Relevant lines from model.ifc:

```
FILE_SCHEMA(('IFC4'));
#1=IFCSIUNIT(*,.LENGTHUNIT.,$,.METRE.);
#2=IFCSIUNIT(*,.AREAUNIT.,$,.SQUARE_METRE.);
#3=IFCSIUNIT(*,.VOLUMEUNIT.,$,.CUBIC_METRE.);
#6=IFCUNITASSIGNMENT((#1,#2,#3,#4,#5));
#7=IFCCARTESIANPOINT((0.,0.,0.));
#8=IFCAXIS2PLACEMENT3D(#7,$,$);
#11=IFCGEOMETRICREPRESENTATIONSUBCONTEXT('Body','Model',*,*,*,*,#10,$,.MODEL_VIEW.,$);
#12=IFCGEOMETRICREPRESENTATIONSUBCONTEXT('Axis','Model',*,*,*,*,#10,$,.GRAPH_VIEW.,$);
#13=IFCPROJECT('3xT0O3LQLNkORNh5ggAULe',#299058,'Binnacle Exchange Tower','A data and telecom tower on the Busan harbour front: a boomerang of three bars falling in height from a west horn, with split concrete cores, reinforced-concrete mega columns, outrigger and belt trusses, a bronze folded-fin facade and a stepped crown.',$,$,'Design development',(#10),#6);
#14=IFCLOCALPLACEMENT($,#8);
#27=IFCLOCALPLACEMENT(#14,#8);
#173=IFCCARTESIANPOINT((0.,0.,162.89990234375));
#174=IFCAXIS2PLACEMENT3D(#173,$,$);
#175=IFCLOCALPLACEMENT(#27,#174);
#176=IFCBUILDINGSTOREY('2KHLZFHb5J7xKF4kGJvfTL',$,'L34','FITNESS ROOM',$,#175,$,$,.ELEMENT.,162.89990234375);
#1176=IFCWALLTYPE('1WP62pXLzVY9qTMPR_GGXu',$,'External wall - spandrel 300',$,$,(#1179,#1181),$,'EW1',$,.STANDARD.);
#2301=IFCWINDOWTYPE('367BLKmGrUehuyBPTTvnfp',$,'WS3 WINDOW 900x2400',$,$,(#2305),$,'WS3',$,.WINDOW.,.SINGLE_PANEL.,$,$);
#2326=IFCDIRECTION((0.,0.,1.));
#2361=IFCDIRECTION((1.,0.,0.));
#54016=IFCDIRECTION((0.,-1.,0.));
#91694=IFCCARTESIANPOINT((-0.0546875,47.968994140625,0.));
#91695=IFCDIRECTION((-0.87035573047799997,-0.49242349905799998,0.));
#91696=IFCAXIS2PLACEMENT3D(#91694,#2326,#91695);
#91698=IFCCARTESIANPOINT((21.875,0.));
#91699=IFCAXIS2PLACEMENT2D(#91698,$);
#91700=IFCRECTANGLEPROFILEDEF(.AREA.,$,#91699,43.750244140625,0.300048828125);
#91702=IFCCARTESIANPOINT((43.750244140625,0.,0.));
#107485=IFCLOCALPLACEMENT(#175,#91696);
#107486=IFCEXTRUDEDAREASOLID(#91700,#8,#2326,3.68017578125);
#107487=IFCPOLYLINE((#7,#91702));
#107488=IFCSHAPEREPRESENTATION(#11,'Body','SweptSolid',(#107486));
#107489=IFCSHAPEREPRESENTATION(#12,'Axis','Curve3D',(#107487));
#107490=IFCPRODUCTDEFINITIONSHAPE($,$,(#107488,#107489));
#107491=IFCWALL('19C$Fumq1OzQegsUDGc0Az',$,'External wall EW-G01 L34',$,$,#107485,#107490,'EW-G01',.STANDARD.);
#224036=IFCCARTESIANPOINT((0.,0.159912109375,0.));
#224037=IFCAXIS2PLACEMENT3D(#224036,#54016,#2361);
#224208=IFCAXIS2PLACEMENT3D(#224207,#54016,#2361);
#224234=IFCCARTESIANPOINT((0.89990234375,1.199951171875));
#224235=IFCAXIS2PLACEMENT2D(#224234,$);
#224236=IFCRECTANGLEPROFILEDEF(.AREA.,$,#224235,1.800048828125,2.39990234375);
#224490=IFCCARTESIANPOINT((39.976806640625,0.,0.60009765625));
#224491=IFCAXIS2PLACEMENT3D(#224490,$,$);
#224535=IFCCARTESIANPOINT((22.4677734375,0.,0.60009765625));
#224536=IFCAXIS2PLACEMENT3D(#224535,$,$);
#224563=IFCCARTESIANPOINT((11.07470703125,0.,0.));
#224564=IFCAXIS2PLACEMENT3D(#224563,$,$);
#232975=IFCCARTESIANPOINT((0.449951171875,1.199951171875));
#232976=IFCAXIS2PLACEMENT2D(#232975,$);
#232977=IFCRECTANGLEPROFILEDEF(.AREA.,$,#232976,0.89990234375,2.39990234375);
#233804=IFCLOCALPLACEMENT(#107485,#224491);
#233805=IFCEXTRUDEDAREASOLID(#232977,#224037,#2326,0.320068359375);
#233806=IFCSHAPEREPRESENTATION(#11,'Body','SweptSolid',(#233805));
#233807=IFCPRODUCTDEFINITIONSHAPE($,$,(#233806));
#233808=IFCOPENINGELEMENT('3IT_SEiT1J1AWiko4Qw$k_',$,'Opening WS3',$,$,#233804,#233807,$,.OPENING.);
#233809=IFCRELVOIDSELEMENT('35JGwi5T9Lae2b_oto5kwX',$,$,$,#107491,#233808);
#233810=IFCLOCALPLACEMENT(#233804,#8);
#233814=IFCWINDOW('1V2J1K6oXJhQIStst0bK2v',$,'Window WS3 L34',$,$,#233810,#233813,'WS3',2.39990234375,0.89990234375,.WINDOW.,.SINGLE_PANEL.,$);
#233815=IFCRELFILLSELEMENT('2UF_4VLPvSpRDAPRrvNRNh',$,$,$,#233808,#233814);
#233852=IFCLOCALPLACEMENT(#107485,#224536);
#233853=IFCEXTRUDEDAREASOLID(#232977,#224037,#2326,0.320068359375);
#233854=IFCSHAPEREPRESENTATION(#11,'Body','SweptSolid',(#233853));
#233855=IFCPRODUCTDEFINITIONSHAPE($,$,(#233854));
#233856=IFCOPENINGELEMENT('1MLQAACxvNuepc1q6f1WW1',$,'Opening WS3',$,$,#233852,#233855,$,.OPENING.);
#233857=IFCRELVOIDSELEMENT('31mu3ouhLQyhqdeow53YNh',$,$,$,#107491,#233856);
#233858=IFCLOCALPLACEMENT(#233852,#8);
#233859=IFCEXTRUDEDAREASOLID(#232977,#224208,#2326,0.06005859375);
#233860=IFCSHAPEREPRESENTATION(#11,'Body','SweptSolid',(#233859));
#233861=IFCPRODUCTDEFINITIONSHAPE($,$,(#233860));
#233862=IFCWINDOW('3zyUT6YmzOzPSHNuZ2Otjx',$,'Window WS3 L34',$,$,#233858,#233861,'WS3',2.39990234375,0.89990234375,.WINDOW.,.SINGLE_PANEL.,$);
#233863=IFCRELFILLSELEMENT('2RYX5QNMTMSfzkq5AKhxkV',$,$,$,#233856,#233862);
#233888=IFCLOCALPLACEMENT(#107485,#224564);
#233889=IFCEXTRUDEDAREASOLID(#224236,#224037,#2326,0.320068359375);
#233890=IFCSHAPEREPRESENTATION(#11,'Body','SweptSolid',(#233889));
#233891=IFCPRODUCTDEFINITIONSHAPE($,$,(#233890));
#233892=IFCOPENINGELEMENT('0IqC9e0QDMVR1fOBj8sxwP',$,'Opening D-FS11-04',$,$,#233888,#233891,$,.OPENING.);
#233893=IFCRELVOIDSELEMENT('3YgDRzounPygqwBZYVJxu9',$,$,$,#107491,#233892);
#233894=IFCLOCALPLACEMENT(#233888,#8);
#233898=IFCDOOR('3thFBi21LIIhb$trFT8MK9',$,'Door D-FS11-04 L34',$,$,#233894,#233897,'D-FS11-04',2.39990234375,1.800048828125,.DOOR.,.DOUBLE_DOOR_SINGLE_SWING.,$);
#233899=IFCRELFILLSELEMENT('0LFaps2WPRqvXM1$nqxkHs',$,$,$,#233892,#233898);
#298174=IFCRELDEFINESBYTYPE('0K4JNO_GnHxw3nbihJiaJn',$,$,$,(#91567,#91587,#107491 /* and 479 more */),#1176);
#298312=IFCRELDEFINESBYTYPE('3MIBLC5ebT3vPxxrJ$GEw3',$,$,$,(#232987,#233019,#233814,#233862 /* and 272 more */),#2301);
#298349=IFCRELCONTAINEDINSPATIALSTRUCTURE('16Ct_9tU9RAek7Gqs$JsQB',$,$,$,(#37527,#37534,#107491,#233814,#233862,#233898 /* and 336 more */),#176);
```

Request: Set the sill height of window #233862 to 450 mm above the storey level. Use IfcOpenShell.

```python
import numpy as np
import ifcopenshell
import ifcopenshell.api.geometry
import ifcopenshell.geom
import ifcopenshell.util.element
import ifcopenshell.util.placement
import ifcopenshell.util.shape
import ifcopenshell.util.unit

model = ifcopenshell.open("model.ifc")
unit_scale = ifcopenshell.util.unit.calculate_unit_scale(model)

window = model.by_id(233862)
opening = window.FillsVoids[0].RelatingOpeningElement
storey = ifcopenshell.util.element.get_container(window, ifc_class="IfcBuildingStorey")
level = ifcopenshell.util.placement.get_local_placement(storey.ObjectPlacement)[2, 3]

# The opening's origin need not be at the sill, so measure its lowest point.
shape = ifcopenshell.geom.create_shape(ifcopenshell.geom.settings(), opening)
bottom = ifcopenshell.util.shape.get_shape_bottom_elevation(shape, shape.geometry) / unit_scale
dz = level + 0.45 - bottom

shift = np.array([0.0, 0.0, dz])
# The window is placed relative to its opening, so it follows when the opening moves.
matrix = ifcopenshell.util.placement.get_local_placement(opening.ObjectPlacement)
matrix[:3, 3] += shift
ifcopenshell.api.geometry.edit_object_placement(
    model, product=opening, matrix=matrix, is_si=False, should_transform_children=True
)

print(f"moved by {dz * unit_scale:+.3f} m")

model.write("model-out.ifc")
```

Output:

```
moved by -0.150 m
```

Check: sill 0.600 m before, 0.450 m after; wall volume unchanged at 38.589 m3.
